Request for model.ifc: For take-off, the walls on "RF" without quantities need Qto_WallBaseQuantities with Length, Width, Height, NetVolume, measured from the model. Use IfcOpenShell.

First a look at what the model holds.

```python
import ifcopenshell
import ifcopenshell.util.element
import ifcopenshell.util.unit

model = ifcopenshell.open("model.ifc")
print(model.schema)
for unit_type in ("LENGTHUNIT", "AREAUNIT", "VOLUMEUNIT"):
    print(unit_type, ifcopenshell.util.unit.calculate_unit_scale(model, unit_type))
storey = next(s for s in model.by_type("IfcBuildingStorey") if s.Name == "RF")
walls = [e for e in ifcopenshell.util.element.get_decomposition(storey) if e.is_a("IfcWall")]
for e in sorted(walls, key=lambda e: e.id()):
    print(e.id(), e.is_a(), e.Name, list(ifcopenshell.util.element.get_psets(e, qtos_only=True)), sep=" | ")
```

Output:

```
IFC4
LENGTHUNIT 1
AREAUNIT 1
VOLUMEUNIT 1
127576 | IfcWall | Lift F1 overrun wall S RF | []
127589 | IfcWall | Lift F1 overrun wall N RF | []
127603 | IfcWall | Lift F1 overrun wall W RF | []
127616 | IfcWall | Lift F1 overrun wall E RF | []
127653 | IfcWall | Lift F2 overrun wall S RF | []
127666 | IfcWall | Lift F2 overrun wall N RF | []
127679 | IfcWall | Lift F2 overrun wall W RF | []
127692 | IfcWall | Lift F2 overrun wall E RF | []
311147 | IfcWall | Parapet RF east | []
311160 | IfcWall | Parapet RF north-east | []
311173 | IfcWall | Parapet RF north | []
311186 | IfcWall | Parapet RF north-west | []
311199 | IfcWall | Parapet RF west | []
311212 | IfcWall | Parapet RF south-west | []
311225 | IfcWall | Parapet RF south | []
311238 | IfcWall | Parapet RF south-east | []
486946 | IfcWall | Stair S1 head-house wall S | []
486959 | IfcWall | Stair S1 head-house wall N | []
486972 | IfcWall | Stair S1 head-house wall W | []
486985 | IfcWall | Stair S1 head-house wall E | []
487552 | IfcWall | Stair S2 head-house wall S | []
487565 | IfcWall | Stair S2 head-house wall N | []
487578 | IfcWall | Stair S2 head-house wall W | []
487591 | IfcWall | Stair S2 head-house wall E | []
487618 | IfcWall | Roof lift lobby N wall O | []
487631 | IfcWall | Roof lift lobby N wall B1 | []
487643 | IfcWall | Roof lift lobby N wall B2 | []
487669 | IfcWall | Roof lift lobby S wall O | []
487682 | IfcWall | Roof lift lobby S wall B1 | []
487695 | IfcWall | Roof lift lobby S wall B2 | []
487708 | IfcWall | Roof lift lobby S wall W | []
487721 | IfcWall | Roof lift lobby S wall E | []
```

```python
import ifcopenshell
import ifcopenshell.api.pset
import ifcopenshell.geom
import ifcopenshell.util.element
import ifcopenshell.util.shape
import ifcopenshell.util.unit

model = ifcopenshell.open("model.ifc")
unit_scale = ifcopenshell.util.unit.calculate_unit_scale(model)
volume_scale = ifcopenshell.util.unit.calculate_unit_scale(model, "VOLUMEUNIT")
settings = ifcopenshell.geom.settings()

storey = next(s for s in model.by_type("IfcBuildingStorey") if s.Name == "RF")
walls = [e for e in ifcopenshell.util.element.get_decomposition(storey) if e.is_a("IfcWall")]

for e in sorted(walls, key=lambda e: e.id()):
    if ifcopenshell.util.element.get_psets(e, qtos_only=True, should_inherit=False):
        continue
    # Geometry comes back in metres, in the element's own axes.
    shape = ifcopenshell.geom.create_shape(settings, e)
    values = {
        "Length": ifcopenshell.util.shape.get_x(shape.geometry) / unit_scale,
        "Width": ifcopenshell.util.shape.get_y(shape.geometry) / unit_scale,
        "Height": ifcopenshell.util.shape.get_z(shape.geometry) / unit_scale,
        "NetVolume": ifcopenshell.util.shape.get_volume(shape.geometry) / volume_scale,
    }
    qto = ifcopenshell.api.pset.add_qto(model, product=e, name="Qto_WallBaseQuantities")
    ifcopenshell.api.pset.edit_qto(model, qto=qto, properties=values)
    print(e.id(), {k: round(v, 3) for k, v in values.items()})

model.write("model_rev.ifc")
```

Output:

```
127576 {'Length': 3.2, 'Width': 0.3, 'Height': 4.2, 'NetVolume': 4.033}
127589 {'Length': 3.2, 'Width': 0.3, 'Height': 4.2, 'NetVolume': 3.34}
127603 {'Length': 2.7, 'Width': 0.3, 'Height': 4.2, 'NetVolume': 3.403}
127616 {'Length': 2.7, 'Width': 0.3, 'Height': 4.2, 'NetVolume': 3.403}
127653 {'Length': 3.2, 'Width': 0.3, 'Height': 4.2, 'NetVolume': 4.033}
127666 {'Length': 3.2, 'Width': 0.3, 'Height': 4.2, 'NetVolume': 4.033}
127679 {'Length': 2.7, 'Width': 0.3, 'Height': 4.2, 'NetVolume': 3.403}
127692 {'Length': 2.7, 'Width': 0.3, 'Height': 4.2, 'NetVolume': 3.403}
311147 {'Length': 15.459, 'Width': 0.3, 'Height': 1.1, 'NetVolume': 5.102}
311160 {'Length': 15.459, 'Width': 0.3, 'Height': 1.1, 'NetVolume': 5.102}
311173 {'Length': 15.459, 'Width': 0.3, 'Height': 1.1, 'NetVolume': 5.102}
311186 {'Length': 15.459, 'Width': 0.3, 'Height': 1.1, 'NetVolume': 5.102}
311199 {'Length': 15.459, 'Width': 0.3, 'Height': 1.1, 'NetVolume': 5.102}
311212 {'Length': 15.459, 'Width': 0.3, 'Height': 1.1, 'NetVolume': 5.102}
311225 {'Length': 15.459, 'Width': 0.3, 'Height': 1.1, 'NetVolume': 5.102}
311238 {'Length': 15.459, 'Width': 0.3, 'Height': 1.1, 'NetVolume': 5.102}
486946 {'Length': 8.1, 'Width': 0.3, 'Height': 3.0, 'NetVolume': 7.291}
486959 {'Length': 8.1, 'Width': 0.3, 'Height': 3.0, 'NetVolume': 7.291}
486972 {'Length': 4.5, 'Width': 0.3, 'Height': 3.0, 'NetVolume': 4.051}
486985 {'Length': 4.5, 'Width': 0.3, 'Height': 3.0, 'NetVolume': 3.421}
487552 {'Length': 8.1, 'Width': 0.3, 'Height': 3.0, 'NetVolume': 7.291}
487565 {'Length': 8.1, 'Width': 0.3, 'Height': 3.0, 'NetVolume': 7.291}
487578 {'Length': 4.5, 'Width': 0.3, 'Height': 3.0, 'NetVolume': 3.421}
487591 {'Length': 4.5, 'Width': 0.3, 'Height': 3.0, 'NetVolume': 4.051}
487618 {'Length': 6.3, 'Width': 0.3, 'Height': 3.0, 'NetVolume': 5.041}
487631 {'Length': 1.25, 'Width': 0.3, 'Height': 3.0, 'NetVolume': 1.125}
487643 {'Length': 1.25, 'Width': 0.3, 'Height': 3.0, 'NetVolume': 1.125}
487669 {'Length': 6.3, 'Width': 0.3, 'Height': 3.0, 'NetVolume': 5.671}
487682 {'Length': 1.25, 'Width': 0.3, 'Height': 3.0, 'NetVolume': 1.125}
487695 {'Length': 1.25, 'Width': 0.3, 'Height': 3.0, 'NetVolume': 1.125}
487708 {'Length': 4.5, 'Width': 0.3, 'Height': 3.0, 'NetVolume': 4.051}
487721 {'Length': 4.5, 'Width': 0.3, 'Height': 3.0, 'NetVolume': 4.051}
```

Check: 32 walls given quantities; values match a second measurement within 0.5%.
